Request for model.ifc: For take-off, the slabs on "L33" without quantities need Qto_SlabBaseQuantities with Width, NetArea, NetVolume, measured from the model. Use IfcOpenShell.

First a look at what the model holds.

```python
import ifcopenshell
import ifcopenshell.util.element
import ifcopenshell.util.unit

model = ifcopenshell.open("model.ifc")
print(model.schema)
for unit_type in ("LENGTHUNIT", "AREAUNIT", "VOLUMEUNIT"):
    print(unit_type, ifcopenshell.util.unit.calculate_unit_scale(model, unit_type))
storey = next(s for s in model.by_type("IfcBuildingStorey") if s.Name == "L33")
slabs = [e for e in ifcopenshell.util.element.get_decomposition(storey) if e.is_a("IfcSlab")]
for e in sorted(slabs, key=lambda e: e.id()):
    print(e.id(), e.is_a(), e.Name, list(ifcopenshell.util.element.get_psets(e, qtos_only=True)), sep=" | ")
```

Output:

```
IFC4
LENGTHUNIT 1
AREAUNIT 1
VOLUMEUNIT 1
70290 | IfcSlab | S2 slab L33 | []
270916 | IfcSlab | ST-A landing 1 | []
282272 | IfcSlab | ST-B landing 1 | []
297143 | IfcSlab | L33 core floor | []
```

```python
import ifcopenshell
import ifcopenshell.api.pset
import ifcopenshell.geom
import ifcopenshell.util.element
import ifcopenshell.util.shape
import ifcopenshell.util.unit

model = ifcopenshell.open("model.ifc")
unit_scale = ifcopenshell.util.unit.calculate_unit_scale(model)
area_scale = ifcopenshell.util.unit.calculate_unit_scale(model, "AREAUNIT")
volume_scale = ifcopenshell.util.unit.calculate_unit_scale(model, "VOLUMEUNIT")
settings = ifcopenshell.geom.settings()

storey = next(s for s in model.by_type("IfcBuildingStorey") if s.Name == "L33")
slabs = [e for e in ifcopenshell.util.element.get_decomposition(storey) if e.is_a("IfcSlab")]

for e in sorted(slabs, key=lambda e: e.id()):
    if ifcopenshell.util.element.get_psets(e, qtos_only=True, should_inherit=False):
        continue
    # Geometry comes back in metres, in the element's own axes.
    shape = ifcopenshell.geom.create_shape(settings, e)
    values = {
        "Width": ifcopenshell.util.shape.get_z(shape.geometry) / unit_scale,
        "NetArea": ifcopenshell.util.shape.get_footprint_area(shape.geometry) / area_scale,
        "NetVolume": ifcopenshell.util.shape.get_volume(shape.geometry) / volume_scale,
    }
    qto = ifcopenshell.api.pset.add_qto(model, product=e, name="Qto_SlabBaseQuantities")
    ifcopenshell.api.pset.edit_qto(model, qto=qto, properties=values)
    print(e.id(), {k: round(v, 3) for k, v in values.items()})

model.write("model_edited.ifc")
```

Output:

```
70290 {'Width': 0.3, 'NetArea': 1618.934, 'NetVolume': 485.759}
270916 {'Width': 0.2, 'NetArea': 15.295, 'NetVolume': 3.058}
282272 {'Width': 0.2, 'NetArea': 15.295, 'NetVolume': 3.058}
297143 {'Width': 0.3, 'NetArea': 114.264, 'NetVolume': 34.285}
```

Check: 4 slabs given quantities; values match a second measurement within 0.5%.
